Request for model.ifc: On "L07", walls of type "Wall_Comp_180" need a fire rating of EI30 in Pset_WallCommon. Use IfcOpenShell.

First a look at what the model holds.

```python
import ifcopenshell
import ifcopenshell.util.element

model = ifcopenshell.open("model.ifc")
print(model.schema)
storey = next(s for s in model.by_type("IfcBuildingStorey") if s.Name == "L07")
walls = [e for e in ifcopenshell.util.element.get_decomposition(storey) if e.is_a("IfcWall")]
seen = {}
for e in walls:
    element_type = ifcopenshell.util.element.get_type(e)
    key = (element_type.Name if element_type != e and element_type else None, ifcopenshell.util.element.get_pset(e, "Pset_WallCommon", "FireRating"))
    seen[key] = seen.get(key, 0) + 1
for (name, value), count in sorted(seen.items(), key=str):
    print(count, "x", name, "|", value)
```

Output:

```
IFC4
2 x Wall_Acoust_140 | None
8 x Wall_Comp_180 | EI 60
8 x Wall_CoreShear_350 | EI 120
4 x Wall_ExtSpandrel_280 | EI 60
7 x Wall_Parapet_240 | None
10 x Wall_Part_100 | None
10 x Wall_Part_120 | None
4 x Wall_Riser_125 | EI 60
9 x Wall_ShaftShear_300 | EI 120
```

```python
import ifcopenshell
import ifcopenshell.api.pset
import ifcopenshell.util.element

model = ifcopenshell.open("model.ifc")

storey = next(s for s in model.by_type("IfcBuildingStorey") if s.Name == "L07")
walls = [e for e in ifcopenshell.util.element.get_decomposition(storey) if e.is_a("IfcWall")]

count = 0
for e in walls:
    element_type = ifcopenshell.util.element.get_type(e)
    if element_type in (None, e) or element_type.Name != "Wall_Comp_180":
        continue
    # add_pset returns the element's existing set when there is one.
    pset = ifcopenshell.api.pset.add_pset(model, product=e, name="Pset_WallCommon")
    ifcopenshell.api.pset.edit_pset(model, pset=pset, properties={"FireRating": "EI30"})
    count += 1

print(count, "walls updated")

model.write("model_rev.ifc")
```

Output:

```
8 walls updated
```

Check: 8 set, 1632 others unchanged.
